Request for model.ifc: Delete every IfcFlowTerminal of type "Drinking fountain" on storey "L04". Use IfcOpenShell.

First a look at what the model holds.

```python
import ifcopenshell
import ifcopenshell.util.element

model = ifcopenshell.open("model.ifc")
print(model.schema)
storey = next(s for s in model.by_type("IfcBuildingStorey") if s.Name == "L04")
terminals = [e for e in ifcopenshell.util.element.get_decomposition(storey) if e.is_a("IfcFlowTerminal")]
seen = {}
for e in terminals:
    element_type = ifcopenshell.util.element.get_type(e)
    name = element_type.Name if element_type not in (None, e) else None
    seen[name] = seen.get(name, 0) + 1
for name, count in sorted(seen.items(), key=str):
    print(count, "x", name)
```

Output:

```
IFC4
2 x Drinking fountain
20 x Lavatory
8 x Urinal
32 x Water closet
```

```python
import ifcopenshell
import ifcopenshell.api.root
import ifcopenshell.util.element

model = ifcopenshell.open("model.ifc")

storey = next(s for s in model.by_type("IfcBuildingStorey") if s.Name == "L04")
terminals = [e for e in ifcopenshell.util.element.get_decomposition(storey) if e.is_a("IfcFlowTerminal")]
targets = [e for e in terminals if (t := ifcopenshell.util.element.get_type(e)) not in (None, e) and t.Name == "Drinking fountain"]

for e in targets:
    ifcopenshell.api.root.remove_product(model, product=e)
print(len(targets), "removed")

model.write("model_v2.ifc")
```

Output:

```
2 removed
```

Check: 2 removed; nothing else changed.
